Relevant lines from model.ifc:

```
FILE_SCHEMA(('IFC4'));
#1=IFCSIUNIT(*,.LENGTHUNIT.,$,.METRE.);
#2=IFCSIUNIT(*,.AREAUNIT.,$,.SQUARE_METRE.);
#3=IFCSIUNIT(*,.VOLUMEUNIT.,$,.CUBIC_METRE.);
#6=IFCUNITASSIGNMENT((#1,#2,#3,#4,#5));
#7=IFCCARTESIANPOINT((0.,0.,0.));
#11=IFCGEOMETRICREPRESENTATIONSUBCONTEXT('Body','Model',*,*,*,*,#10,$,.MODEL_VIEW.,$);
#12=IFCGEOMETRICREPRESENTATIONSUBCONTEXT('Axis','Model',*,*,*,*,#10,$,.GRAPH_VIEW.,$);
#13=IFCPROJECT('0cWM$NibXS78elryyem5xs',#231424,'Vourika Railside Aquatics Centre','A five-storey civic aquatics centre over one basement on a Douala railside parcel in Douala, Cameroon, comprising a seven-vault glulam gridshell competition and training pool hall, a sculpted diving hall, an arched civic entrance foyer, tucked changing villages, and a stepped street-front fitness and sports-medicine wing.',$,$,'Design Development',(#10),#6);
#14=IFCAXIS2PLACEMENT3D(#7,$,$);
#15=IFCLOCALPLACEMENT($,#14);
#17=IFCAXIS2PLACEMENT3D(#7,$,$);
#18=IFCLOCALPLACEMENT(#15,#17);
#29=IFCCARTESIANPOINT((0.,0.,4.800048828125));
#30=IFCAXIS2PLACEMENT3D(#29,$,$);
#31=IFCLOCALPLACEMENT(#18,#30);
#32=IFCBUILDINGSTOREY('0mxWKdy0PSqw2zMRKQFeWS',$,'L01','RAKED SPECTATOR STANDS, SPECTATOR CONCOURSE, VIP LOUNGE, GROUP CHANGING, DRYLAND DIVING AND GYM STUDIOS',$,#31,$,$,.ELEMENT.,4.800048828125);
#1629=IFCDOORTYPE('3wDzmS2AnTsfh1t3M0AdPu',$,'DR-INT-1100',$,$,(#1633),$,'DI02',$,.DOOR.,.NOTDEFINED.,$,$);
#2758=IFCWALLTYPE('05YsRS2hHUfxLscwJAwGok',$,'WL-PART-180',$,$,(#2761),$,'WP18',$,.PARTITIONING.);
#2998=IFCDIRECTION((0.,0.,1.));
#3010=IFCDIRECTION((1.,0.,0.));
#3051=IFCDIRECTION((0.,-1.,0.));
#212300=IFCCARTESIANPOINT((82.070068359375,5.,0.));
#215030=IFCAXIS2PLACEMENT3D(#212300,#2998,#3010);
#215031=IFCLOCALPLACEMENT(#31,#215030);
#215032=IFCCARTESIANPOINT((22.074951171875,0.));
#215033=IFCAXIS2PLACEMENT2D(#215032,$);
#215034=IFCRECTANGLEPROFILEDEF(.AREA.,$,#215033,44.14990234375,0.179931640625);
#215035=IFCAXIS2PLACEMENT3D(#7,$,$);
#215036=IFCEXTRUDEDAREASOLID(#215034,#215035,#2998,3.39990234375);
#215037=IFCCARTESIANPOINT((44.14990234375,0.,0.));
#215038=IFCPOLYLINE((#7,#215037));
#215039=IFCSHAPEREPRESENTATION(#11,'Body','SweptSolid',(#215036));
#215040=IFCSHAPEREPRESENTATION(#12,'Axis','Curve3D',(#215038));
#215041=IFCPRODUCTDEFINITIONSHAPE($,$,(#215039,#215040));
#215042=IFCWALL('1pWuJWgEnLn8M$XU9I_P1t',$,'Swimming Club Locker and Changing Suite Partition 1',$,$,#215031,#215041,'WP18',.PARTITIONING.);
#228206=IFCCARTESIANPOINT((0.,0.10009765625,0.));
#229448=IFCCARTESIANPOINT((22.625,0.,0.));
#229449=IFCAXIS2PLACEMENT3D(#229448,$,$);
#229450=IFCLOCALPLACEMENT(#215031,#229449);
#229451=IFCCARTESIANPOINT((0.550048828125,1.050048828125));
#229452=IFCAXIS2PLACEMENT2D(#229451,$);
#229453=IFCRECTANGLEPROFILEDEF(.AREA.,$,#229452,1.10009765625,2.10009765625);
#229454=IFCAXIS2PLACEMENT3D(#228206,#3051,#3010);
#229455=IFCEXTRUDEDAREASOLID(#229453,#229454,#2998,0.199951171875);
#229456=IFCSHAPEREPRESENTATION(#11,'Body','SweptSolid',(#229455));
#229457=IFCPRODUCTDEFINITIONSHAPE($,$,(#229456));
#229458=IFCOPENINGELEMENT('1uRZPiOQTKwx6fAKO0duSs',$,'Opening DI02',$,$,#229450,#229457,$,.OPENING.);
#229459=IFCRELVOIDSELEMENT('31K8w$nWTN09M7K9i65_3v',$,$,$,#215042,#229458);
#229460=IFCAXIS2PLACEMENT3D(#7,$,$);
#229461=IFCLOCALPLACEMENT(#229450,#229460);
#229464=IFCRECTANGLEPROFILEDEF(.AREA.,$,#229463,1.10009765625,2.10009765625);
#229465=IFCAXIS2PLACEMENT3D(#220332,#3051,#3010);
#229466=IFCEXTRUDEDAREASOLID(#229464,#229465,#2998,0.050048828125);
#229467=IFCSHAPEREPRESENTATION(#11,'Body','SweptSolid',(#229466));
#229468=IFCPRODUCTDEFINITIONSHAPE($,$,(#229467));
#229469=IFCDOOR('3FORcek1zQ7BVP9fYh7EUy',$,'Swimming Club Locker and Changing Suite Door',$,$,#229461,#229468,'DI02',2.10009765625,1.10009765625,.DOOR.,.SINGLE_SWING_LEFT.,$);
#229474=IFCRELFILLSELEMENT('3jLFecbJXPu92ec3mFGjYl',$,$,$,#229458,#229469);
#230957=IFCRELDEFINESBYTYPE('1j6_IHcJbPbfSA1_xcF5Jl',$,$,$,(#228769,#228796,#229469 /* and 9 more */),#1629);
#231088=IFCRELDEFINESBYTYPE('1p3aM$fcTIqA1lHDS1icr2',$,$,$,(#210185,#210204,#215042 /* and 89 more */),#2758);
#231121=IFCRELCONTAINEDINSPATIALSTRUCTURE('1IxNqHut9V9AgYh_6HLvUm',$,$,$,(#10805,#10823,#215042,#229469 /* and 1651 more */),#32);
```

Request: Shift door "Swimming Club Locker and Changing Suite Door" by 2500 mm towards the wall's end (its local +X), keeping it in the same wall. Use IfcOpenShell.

```python
import ifcopenshell
import ifcopenshell.api.geometry
import ifcopenshell.util.placement
import ifcopenshell.util.unit

model = ifcopenshell.open("model.ifc")
unit_scale = ifcopenshell.util.unit.calculate_unit_scale(model)

door = model.by_guid("3FORcek1zQ7BVP9fYh7EUy")
opening = door.FillsVoids[0].RelatingOpeningElement
wall = opening.VoidsElements[0].RelatingBuildingElement

wall_matrix = ifcopenshell.util.placement.get_local_placement(wall.ObjectPlacement)
shift = wall_matrix[:3, 0] * 2.5 / unit_scale
before = ifcopenshell.util.placement.get_local_placement(door.ObjectPlacement)[:3, 3].copy()

# The door is placed relative to its opening, so it follows when the opening moves.
matrix = ifcopenshell.util.placement.get_local_placement(opening.ObjectPlacement)
matrix[:3, 3] += shift
ifcopenshell.api.geometry.edit_object_placement(
    model, product=opening, matrix=matrix, is_si=False, should_transform_children=True
)

after = ifcopenshell.util.placement.get_local_placement(door.ObjectPlacement)[:3, 3]
print("door moved by", (after - before).round(3) + 0.0)

model.write("model_rev.ifc")
```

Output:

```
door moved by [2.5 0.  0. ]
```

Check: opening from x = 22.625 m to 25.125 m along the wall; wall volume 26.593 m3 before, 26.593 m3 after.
